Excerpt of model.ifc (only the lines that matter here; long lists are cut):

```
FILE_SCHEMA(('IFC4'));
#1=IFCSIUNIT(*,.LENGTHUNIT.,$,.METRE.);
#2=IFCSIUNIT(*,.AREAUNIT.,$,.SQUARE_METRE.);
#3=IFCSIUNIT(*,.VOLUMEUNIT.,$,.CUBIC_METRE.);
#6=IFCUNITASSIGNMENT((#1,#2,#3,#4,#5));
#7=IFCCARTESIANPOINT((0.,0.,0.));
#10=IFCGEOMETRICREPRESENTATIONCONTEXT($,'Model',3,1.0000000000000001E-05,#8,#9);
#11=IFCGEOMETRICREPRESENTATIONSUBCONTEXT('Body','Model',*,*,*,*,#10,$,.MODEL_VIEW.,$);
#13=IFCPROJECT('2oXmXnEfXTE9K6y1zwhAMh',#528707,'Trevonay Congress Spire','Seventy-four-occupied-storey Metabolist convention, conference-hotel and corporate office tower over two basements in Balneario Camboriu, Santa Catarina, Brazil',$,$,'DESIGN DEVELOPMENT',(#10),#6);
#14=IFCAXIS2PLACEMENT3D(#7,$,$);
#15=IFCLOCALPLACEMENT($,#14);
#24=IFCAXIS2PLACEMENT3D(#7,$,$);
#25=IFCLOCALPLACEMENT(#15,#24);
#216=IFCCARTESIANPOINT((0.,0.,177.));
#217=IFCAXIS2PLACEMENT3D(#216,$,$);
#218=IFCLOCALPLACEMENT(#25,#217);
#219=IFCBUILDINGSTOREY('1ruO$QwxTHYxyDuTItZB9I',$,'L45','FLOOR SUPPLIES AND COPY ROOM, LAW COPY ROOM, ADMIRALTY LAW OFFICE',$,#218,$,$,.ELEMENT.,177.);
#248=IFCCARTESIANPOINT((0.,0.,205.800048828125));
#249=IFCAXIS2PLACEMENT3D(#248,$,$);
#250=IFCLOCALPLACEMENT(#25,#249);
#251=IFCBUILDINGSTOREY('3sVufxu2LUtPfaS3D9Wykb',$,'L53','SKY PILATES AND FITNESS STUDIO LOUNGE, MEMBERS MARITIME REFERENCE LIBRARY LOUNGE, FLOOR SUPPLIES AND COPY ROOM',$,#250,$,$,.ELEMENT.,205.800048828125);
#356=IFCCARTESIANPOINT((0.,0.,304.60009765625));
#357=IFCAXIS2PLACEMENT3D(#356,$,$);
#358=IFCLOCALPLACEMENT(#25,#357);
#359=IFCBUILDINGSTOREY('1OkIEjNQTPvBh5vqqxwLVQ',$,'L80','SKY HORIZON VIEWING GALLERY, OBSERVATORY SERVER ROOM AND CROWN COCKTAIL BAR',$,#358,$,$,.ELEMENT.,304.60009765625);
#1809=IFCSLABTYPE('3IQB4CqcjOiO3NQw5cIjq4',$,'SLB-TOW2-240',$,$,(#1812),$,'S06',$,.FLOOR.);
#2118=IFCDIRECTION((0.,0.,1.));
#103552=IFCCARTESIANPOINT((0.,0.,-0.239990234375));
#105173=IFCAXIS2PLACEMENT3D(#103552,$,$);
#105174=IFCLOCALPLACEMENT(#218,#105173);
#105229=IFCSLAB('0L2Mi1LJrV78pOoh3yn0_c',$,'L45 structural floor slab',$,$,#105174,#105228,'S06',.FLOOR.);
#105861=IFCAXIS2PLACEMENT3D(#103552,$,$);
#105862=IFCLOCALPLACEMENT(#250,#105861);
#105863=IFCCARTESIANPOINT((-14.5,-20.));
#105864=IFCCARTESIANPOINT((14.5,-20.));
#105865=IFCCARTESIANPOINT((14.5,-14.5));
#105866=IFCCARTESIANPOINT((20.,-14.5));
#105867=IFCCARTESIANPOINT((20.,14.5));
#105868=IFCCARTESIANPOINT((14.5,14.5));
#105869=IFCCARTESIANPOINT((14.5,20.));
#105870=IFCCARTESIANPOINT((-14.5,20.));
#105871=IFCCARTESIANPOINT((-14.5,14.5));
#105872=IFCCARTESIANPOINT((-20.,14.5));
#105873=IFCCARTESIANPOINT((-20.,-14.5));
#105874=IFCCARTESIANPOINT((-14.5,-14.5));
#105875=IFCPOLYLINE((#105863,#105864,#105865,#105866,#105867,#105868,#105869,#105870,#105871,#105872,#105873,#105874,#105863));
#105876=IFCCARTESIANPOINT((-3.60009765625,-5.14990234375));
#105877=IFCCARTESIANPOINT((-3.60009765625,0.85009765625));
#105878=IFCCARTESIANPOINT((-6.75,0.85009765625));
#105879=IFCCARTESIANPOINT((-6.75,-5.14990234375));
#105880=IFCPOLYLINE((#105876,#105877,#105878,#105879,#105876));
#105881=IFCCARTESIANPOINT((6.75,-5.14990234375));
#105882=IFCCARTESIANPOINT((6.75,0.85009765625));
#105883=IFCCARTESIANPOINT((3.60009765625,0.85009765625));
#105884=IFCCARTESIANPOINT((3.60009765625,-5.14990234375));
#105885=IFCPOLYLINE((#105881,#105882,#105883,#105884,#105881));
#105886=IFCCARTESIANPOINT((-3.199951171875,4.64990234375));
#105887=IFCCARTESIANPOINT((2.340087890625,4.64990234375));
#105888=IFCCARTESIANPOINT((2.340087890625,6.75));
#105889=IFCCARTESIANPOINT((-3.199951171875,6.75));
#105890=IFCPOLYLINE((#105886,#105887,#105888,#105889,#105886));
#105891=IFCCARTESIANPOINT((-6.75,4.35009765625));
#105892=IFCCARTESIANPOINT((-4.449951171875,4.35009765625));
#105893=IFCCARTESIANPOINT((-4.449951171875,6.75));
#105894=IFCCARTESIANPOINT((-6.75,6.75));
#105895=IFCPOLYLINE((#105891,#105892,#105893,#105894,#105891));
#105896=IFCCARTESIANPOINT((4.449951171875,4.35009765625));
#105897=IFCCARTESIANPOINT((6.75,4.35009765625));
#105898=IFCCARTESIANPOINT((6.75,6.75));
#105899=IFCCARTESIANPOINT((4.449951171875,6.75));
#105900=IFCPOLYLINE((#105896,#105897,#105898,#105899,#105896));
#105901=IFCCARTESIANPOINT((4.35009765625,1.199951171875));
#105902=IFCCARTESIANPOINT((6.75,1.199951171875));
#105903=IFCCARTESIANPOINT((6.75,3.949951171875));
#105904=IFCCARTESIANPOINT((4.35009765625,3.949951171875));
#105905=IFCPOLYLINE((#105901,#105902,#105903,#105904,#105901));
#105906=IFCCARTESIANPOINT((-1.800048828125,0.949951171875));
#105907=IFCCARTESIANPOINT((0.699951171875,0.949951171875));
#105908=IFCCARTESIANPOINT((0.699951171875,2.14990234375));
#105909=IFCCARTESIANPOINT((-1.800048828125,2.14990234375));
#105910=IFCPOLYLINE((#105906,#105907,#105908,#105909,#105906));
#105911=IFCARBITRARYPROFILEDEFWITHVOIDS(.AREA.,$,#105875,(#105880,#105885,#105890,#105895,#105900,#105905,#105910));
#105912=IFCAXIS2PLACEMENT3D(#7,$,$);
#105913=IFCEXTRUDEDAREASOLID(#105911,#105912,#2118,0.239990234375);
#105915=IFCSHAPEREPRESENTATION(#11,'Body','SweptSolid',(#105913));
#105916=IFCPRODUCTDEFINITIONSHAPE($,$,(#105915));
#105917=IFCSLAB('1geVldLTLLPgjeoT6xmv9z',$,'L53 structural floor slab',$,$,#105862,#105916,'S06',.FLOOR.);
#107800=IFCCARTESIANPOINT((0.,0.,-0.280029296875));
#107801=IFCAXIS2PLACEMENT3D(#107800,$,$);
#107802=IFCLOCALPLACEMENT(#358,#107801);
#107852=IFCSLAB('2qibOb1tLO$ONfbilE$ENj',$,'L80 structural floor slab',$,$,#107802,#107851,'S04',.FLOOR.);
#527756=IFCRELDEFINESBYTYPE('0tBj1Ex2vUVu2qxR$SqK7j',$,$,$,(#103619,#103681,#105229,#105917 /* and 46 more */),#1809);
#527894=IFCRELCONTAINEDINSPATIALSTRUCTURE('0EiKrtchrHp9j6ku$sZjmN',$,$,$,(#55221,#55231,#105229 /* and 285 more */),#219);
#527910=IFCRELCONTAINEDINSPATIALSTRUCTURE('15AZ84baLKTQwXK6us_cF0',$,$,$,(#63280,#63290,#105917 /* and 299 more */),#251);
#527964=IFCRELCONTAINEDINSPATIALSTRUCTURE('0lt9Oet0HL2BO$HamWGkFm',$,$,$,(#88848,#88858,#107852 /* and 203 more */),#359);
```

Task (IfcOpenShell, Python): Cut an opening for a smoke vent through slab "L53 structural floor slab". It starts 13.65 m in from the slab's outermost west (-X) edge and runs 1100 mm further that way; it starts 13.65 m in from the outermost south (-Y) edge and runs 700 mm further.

```python
import numpy as np
import ifcopenshell
import ifcopenshell.api.feature
import ifcopenshell.api.geometry
import ifcopenshell.api.root
import ifcopenshell.geom
import ifcopenshell.util.placement
import ifcopenshell.util.representation
import ifcopenshell.util.shape
import ifcopenshell.util.unit

model = ifcopenshell.open("model.ifc")
unit_scale = ifcopenshell.util.unit.calculate_unit_scale(model)
settings = ifcopenshell.geom.settings()


def volume(element):
    """Net volume in cubic metres, openings subtracted."""
    shape = ifcopenshell.geom.create_shape(settings, element)
    return ifcopenshell.util.shape.get_volume(shape.geometry)


slab = model.by_guid("1geVldLTLLPgjeoT6xmv9z")
before = volume(slab)

# Extent in the slab's own axes, in metres. The edges named are its -X and -Y sides.
slab_shape = ifcopenshell.geom.create_shape(settings, slab)
vertices = ifcopenshell.util.shape.get_vertices(slab_shape.geometry)
x_min, y_min, bottom = vertices.min(axis=0)
top = vertices[:, 2].max()

opening = ifcopenshell.api.root.create_entity(model, ifc_class="IfcOpeningElement", name="Smoke vent opening", predefined_type="OPENING")
context = ifcopenshell.util.representation.get_context(model, "Model", "Body", "MODEL_VIEW")
width, depth = 1.1, 0.7
outline = [(0.0, 0.0), (width, 0.0), (width, depth), (0.0, depth), (0.0, 0.0)]
# Overshoot both faces by 50 mm so the cut is clean.
shape = ifcopenshell.api.geometry.add_slab_representation(
    model, context=context, depth=top - bottom + 0.1, polyline=outline
)
ifcopenshell.api.geometry.assign_representation(model, product=opening, representation=shape)

matrix = ifcopenshell.util.placement.get_local_placement(slab.ObjectPlacement)
matrix[:, 3] = matrix @ np.append(np.array([x_min + 13.65, y_min + 13.65, bottom - 0.05]) / unit_scale, 1.0)
ifcopenshell.api.geometry.edit_object_placement(model, product=opening, matrix=matrix, is_si=False)
ifcopenshell.api.feature.add_feature(model, feature=opening, element=slab)

after = volume(slab)

print(f"slab volume {before:.3f} -> {after:.3f} m3")

model.write("model-out.ifc")
```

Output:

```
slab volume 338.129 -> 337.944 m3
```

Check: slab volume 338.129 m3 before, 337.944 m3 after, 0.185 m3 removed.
